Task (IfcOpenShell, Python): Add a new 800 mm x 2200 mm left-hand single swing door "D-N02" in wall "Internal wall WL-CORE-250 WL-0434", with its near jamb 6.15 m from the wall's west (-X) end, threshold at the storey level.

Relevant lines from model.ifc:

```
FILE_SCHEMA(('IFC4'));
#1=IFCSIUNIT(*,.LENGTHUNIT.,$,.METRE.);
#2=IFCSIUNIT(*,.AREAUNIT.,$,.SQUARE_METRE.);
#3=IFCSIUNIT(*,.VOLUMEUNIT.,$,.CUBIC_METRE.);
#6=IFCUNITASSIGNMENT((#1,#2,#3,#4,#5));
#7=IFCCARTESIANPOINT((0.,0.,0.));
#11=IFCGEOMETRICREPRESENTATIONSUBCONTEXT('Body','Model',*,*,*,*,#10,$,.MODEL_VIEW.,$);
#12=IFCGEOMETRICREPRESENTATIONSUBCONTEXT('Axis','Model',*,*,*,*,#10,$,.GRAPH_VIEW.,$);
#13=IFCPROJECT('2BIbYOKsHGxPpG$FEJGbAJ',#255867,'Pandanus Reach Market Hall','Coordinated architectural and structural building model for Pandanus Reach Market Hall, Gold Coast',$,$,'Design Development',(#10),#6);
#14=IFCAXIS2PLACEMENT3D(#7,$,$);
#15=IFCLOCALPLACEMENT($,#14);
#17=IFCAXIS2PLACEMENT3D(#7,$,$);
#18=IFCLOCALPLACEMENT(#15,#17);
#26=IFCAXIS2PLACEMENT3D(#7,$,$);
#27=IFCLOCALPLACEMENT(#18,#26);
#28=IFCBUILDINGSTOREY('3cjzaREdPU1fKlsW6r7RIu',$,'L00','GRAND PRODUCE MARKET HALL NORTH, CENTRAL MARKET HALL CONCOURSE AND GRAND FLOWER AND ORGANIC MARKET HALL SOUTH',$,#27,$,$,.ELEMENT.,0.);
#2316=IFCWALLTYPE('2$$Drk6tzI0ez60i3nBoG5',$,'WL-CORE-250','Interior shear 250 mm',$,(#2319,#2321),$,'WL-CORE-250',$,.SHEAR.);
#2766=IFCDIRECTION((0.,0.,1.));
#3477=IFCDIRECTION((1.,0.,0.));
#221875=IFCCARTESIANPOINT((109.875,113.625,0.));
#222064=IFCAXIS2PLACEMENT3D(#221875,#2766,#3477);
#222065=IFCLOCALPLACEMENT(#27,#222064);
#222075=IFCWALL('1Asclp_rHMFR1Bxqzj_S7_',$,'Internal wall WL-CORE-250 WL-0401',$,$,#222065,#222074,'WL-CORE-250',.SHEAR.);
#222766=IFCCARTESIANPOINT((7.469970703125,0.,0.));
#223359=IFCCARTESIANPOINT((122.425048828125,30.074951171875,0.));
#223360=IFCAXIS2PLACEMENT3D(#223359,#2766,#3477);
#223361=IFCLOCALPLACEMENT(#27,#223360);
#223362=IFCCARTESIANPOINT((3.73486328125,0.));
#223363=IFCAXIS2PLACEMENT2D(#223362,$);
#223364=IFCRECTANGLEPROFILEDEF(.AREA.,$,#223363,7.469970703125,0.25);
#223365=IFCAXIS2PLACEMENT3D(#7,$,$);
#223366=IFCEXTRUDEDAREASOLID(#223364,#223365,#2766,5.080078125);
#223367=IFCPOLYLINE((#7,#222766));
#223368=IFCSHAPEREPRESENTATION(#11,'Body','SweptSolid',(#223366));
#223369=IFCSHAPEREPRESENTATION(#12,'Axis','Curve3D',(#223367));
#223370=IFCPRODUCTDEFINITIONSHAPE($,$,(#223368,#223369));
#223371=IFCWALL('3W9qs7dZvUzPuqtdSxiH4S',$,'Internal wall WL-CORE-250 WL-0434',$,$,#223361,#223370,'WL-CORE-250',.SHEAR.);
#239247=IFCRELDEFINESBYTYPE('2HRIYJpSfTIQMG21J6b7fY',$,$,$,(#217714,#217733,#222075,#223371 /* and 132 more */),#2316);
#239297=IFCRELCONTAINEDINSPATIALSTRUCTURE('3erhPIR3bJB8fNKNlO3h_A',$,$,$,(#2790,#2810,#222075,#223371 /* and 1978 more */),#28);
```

```python
import numpy as np
import ifcopenshell
import ifcopenshell.api.feature
import ifcopenshell.api.geometry
import ifcopenshell.api.root
import ifcopenshell.api.spatial
import ifcopenshell.geom
import ifcopenshell.util.element
import ifcopenshell.util.placement
import ifcopenshell.util.representation
import ifcopenshell.util.shape
import ifcopenshell.util.unit

model = ifcopenshell.open("model.ifc")
unit_scale = ifcopenshell.util.unit.calculate_unit_scale(model)
settings = ifcopenshell.geom.settings()


def volume(element):
    """Net volume in cubic metres, openings subtracted."""
    shape = ifcopenshell.geom.create_shape(settings, element)
    return ifcopenshell.util.shape.get_volume(shape.geometry)


wall = model.by_guid("3W9qs7dZvUzPuqtdSxiH4S")
storey = ifcopenshell.util.element.get_container(wall, ifc_class="IfcBuildingStorey")
context = ifcopenshell.util.representation.get_context(model, "Model", "Body", "MODEL_VIEW")
before = volume(wall)

width, height, from_end, sill = 0.8, 2.2, 6.15, 0.0  # metres

# The wall runs along its own X axis, and the end named is its -X end.
wall_shape = ifcopenshell.geom.create_shape(settings, wall)
x, y, z = ifcopenshell.util.shape.get_vertices(wall_shape.geometry).T
start = x.min() + from_end
face, thickness = float(y.min()), float(y.max() - y.min())
wall_matrix = ifcopenshell.util.placement.get_local_placement(wall.ObjectPlacement)
level = ifcopenshell.util.placement.get_local_placement(storey.ObjectPlacement)[2, 3]


def in_wall(x, y):
    """Placement at x, y metres in the wall's axes, at sill height."""
    matrix = wall_matrix.copy()
    matrix[:, 3] = wall_matrix @ np.array([x / unit_scale, y / unit_scale, 0.0, 1.0])
    matrix[2, 3] = level + sill / unit_scale
    return matrix


# Opening: a box that overshoots both wall faces by 50 mm.
opening = ifcopenshell.api.root.create_entity(model, ifc_class="IfcOpeningElement", predefined_type="OPENING")
box = ifcopenshell.api.geometry.add_wall_representation(
    model, context=context, length=width, height=height, thickness=thickness + 0.1
)
ifcopenshell.api.geometry.assign_representation(model, product=opening, representation=box)
ifcopenshell.api.geometry.edit_object_placement(model, product=opening, matrix=in_wall(start, face - 0.05), is_si=False)
ifcopenshell.api.feature.add_feature(model, feature=opening, element=wall)

door = ifcopenshell.api.root.create_entity(model, ifc_class="IfcDoor", name="D-N02", predefined_type="DOOR")
door.OverallWidth, door.OverallHeight = width / unit_scale, height / unit_scale
door.OperationType = "SINGLE_SWING_LEFT"
body = ifcopenshell.api.geometry.add_door_representation(
    model,
    context=context,
    overall_width=door.OverallWidth,
    overall_height=door.OverallHeight,
    operation_type="SINGLE_SWING_LEFT",
    lining_properties={"LiningDepth": thickness / unit_scale, "ThresholdDepth": thickness / unit_scale},
)
ifcopenshell.api.geometry.assign_representation(model, product=door, representation=body)
ifcopenshell.api.spatial.assign_container(model, products=[door], relating_structure=storey)
ifcopenshell.api.feature.add_filling(model, opening=opening, element=door)

# The lining spans the wall, so the door starts at the wall face.
ifcopenshell.api.geometry.edit_object_placement(model, product=door, matrix=in_wall(start, face), is_si=False)

after = volume(wall)

print(f"wall volume {before:.3f} -> {after:.3f} m3")

model.write("model_v2.ifc")
```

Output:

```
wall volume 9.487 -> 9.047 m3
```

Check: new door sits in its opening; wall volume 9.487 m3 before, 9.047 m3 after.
